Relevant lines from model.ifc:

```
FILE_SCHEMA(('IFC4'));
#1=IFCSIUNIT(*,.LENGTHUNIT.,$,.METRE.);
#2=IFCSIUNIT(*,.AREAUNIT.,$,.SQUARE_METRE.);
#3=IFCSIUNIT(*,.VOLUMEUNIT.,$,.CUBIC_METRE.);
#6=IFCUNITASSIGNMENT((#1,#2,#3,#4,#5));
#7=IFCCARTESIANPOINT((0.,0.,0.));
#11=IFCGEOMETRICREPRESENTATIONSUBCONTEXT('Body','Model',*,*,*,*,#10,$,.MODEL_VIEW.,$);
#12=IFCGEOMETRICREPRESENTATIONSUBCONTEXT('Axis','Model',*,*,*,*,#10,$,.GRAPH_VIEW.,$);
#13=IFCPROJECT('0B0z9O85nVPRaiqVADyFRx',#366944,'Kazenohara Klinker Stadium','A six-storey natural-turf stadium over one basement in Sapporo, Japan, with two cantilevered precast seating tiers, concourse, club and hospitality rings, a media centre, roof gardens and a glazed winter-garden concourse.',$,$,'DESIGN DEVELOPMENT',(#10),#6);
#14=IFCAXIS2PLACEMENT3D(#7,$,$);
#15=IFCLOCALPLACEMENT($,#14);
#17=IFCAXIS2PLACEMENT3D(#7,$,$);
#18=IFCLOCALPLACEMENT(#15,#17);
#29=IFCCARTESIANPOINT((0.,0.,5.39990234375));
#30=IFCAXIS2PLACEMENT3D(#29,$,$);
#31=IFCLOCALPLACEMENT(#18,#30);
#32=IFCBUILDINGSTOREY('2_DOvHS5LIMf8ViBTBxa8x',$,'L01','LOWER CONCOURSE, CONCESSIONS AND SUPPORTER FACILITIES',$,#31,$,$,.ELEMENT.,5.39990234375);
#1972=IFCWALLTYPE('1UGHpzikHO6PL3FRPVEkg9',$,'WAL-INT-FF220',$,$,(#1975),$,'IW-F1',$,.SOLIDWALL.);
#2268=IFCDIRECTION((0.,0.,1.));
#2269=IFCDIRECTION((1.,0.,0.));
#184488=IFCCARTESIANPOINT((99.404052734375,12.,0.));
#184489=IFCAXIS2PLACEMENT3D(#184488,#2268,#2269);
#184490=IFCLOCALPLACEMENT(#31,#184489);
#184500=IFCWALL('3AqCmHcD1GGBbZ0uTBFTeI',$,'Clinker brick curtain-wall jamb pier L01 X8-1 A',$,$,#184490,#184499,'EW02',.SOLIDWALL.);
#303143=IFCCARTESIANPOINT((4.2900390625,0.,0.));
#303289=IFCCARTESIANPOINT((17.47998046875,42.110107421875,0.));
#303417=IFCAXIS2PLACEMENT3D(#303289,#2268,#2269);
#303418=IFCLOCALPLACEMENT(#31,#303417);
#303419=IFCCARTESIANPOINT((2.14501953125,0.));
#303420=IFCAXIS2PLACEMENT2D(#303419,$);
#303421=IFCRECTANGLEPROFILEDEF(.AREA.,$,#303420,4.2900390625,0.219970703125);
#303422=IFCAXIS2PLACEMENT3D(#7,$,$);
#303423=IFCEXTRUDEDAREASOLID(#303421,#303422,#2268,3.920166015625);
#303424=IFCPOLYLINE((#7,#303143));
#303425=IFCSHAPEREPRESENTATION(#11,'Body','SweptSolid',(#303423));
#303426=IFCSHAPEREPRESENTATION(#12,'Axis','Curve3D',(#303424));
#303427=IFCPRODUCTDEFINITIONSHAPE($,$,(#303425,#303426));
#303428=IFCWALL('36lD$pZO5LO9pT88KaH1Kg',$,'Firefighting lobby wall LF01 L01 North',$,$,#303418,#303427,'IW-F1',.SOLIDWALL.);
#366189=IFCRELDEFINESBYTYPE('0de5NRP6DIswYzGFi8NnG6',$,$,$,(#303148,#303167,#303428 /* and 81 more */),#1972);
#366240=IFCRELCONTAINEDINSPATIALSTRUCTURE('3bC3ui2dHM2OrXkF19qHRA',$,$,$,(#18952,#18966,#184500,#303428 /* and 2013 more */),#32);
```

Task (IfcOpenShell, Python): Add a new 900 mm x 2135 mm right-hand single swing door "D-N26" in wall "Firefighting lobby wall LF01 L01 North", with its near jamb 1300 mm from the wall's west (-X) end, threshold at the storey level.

```python
import numpy as np
import ifcopenshell
import ifcopenshell.api.feature
import ifcopenshell.api.geometry
import ifcopenshell.api.root
import ifcopenshell.api.spatial
import ifcopenshell.geom
import ifcopenshell.util.element
import ifcopenshell.util.placement
import ifcopenshell.util.representation
import ifcopenshell.util.shape
import ifcopenshell.util.unit

model = ifcopenshell.open("model.ifc")
unit_scale = ifcopenshell.util.unit.calculate_unit_scale(model)
settings = ifcopenshell.geom.settings()


def volume(element):
    """Net volume in cubic metres, openings subtracted."""
    shape = ifcopenshell.geom.create_shape(settings, element)
    return ifcopenshell.util.shape.get_volume(shape.geometry)


wall = model.by_guid("36lD$pZO5LO9pT88KaH1Kg")
storey = ifcopenshell.util.element.get_container(wall, ifc_class="IfcBuildingStorey")
context = ifcopenshell.util.representation.get_context(model, "Model", "Body", "MODEL_VIEW")
before = volume(wall)

width, height, from_end, sill = 0.9, 2.135, 1.3, 0.0  # metres

# The wall runs along its own X axis, and the end named is its -X end.
wall_shape = ifcopenshell.geom.create_shape(settings, wall)
x, y, z = ifcopenshell.util.shape.get_vertices(wall_shape.geometry).T
start = x.min() + from_end
face, thickness = float(y.min()), float(y.max() - y.min())
wall_matrix = ifcopenshell.util.placement.get_local_placement(wall.ObjectPlacement)
level = ifcopenshell.util.placement.get_local_placement(storey.ObjectPlacement)[2, 3]


def in_wall(x, y):
    """Placement at x, y metres in the wall's axes, at sill height."""
    matrix = wall_matrix.copy()
    matrix[:, 3] = wall_matrix @ np.array([x / unit_scale, y / unit_scale, 0.0, 1.0])
    matrix[2, 3] = level + sill / unit_scale
    return matrix


# Opening: a box that overshoots both wall faces by 50 mm.
opening = ifcopenshell.api.root.create_entity(model, ifc_class="IfcOpeningElement", predefined_type="OPENING")
box = ifcopenshell.api.geometry.add_wall_representation(
    model, context=context, length=width, height=height, thickness=thickness + 0.1
)
ifcopenshell.api.geometry.assign_representation(model, product=opening, representation=box)
ifcopenshell.api.geometry.edit_object_placement(model, product=opening, matrix=in_wall(start, face - 0.05), is_si=False)
ifcopenshell.api.feature.add_feature(model, feature=opening, element=wall)

door = ifcopenshell.api.root.create_entity(model, ifc_class="IfcDoor", name="D-N26", predefined_type="DOOR")
door.OverallWidth, door.OverallHeight = width / unit_scale, height / unit_scale
door.OperationType = "SINGLE_SWING_RIGHT"
body = ifcopenshell.api.geometry.add_door_representation(
    model,
    context=context,
    overall_width=door.OverallWidth,
    overall_height=door.OverallHeight,
    operation_type="SINGLE_SWING_RIGHT",
    lining_properties={"LiningDepth": thickness / unit_scale, "ThresholdDepth": thickness / unit_scale},
)
ifcopenshell.api.geometry.assign_representation(model, product=door, representation=body)
ifcopenshell.api.spatial.assign_container(model, products=[door], relating_structure=storey)
ifcopenshell.api.feature.add_filling(model, opening=opening, element=door)

# The lining spans the wall, so the door starts at the wall face.
ifcopenshell.api.geometry.edit_object_placement(model, product=door, matrix=in_wall(start, face), is_si=False)

after = volume(wall)

print(f"wall volume {before:.3f} -> {after:.3f} m3")

model.write("model_edited.ifc")
```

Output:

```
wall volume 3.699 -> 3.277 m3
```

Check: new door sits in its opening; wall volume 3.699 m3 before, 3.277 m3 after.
